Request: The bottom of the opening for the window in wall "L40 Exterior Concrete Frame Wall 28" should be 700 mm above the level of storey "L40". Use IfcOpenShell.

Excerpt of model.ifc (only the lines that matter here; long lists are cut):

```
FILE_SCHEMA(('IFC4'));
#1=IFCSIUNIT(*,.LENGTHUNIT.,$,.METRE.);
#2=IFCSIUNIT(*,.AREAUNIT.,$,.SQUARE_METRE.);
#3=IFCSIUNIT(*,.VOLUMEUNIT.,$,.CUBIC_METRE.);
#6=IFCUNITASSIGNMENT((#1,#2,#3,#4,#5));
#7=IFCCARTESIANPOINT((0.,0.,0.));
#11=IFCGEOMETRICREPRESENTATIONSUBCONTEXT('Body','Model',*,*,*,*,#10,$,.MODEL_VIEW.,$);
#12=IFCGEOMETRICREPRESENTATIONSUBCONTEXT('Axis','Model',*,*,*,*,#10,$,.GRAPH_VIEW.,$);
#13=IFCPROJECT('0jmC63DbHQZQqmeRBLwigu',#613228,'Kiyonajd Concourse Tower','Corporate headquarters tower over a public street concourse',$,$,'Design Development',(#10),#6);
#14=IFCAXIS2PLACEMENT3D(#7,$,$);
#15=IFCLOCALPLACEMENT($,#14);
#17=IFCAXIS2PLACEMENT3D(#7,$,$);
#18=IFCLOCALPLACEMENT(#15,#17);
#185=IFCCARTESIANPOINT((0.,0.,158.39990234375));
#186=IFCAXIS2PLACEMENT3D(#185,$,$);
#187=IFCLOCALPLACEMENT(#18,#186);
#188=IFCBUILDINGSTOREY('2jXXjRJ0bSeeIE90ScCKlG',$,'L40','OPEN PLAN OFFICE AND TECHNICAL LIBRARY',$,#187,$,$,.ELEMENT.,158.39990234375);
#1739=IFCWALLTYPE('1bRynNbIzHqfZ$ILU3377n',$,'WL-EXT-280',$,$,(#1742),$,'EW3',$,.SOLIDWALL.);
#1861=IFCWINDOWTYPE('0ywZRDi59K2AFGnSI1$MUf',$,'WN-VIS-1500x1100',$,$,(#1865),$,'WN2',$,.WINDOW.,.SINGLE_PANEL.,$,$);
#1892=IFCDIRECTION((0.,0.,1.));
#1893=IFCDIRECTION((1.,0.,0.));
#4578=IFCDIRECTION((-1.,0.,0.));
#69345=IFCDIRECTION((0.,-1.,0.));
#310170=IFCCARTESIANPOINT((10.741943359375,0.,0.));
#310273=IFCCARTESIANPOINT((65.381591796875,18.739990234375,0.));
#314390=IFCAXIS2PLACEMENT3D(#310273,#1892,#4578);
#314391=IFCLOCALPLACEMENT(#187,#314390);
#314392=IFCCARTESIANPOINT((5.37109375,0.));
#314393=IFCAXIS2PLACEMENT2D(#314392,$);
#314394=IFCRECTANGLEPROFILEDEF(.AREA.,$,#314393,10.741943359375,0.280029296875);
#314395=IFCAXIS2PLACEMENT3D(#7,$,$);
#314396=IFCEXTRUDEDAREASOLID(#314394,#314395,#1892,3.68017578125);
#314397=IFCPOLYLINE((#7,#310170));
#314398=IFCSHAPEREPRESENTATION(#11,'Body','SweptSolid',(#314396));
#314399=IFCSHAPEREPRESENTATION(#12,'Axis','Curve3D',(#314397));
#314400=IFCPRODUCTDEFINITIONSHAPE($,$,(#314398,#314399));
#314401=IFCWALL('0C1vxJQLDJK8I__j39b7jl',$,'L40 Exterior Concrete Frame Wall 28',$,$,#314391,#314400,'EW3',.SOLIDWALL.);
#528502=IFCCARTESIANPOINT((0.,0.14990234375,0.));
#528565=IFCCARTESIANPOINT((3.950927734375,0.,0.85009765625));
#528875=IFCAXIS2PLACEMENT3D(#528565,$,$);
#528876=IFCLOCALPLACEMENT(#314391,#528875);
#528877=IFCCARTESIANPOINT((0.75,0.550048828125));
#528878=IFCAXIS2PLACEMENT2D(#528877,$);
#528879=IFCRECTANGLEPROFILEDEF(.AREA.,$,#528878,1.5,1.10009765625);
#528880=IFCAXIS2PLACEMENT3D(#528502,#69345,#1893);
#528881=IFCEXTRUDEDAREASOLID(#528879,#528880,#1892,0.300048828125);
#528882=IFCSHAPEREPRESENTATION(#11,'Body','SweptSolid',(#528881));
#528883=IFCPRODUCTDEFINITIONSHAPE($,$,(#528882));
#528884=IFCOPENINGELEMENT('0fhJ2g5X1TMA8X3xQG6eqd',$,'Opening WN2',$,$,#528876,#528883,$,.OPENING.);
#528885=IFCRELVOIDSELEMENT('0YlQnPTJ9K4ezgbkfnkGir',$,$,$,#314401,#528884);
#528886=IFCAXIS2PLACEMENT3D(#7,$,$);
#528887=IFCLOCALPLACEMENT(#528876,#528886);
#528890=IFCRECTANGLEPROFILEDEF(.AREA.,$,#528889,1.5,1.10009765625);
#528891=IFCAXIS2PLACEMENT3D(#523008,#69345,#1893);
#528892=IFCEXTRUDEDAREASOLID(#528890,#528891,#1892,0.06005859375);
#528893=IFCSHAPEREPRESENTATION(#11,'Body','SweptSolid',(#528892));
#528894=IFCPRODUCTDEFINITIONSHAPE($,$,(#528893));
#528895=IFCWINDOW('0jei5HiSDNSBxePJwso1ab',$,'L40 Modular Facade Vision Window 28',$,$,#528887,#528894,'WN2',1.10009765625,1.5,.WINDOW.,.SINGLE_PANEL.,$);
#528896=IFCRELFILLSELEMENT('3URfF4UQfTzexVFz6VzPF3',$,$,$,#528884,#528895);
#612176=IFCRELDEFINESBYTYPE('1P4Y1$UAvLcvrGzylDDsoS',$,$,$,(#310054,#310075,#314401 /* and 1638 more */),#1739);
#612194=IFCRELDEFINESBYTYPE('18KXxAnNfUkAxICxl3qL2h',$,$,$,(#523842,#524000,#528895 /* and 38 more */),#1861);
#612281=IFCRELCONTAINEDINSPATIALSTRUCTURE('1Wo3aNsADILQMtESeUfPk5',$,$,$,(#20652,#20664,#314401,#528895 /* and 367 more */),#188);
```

```python
import numpy as np
import ifcopenshell
import ifcopenshell.api.geometry
import ifcopenshell.geom
import ifcopenshell.util.element
import ifcopenshell.util.placement
import ifcopenshell.util.shape
import ifcopenshell.util.unit

model = ifcopenshell.open("model.ifc")
unit_scale = ifcopenshell.util.unit.calculate_unit_scale(model)

window = model.by_guid("0jei5HiSDNSBxePJwso1ab")
opening = window.FillsVoids[0].RelatingOpeningElement
storey = ifcopenshell.util.element.get_container(window, ifc_class="IfcBuildingStorey")
level = ifcopenshell.util.placement.get_local_placement(storey.ObjectPlacement)[2, 3]

# The opening's origin need not be at the sill, so measure its lowest point.
shape = ifcopenshell.geom.create_shape(ifcopenshell.geom.settings(), opening)
bottom = ifcopenshell.util.shape.get_shape_bottom_elevation(shape, shape.geometry) / unit_scale
dz = level + 0.7 / unit_scale - bottom

shift = np.array([0.0, 0.0, dz])
# The window is placed relative to its opening, so it follows when the opening moves.
matrix = ifcopenshell.util.placement.get_local_placement(opening.ObjectPlacement)
matrix[:3, 3] += shift
ifcopenshell.api.geometry.edit_object_placement(
    model, product=opening, matrix=matrix, is_si=False, should_transform_children=True
)

print(f"moved by {dz * unit_scale:+.3f} m")

model.write("model_updated.ifc")
```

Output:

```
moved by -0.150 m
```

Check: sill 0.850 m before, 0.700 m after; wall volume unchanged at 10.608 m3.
